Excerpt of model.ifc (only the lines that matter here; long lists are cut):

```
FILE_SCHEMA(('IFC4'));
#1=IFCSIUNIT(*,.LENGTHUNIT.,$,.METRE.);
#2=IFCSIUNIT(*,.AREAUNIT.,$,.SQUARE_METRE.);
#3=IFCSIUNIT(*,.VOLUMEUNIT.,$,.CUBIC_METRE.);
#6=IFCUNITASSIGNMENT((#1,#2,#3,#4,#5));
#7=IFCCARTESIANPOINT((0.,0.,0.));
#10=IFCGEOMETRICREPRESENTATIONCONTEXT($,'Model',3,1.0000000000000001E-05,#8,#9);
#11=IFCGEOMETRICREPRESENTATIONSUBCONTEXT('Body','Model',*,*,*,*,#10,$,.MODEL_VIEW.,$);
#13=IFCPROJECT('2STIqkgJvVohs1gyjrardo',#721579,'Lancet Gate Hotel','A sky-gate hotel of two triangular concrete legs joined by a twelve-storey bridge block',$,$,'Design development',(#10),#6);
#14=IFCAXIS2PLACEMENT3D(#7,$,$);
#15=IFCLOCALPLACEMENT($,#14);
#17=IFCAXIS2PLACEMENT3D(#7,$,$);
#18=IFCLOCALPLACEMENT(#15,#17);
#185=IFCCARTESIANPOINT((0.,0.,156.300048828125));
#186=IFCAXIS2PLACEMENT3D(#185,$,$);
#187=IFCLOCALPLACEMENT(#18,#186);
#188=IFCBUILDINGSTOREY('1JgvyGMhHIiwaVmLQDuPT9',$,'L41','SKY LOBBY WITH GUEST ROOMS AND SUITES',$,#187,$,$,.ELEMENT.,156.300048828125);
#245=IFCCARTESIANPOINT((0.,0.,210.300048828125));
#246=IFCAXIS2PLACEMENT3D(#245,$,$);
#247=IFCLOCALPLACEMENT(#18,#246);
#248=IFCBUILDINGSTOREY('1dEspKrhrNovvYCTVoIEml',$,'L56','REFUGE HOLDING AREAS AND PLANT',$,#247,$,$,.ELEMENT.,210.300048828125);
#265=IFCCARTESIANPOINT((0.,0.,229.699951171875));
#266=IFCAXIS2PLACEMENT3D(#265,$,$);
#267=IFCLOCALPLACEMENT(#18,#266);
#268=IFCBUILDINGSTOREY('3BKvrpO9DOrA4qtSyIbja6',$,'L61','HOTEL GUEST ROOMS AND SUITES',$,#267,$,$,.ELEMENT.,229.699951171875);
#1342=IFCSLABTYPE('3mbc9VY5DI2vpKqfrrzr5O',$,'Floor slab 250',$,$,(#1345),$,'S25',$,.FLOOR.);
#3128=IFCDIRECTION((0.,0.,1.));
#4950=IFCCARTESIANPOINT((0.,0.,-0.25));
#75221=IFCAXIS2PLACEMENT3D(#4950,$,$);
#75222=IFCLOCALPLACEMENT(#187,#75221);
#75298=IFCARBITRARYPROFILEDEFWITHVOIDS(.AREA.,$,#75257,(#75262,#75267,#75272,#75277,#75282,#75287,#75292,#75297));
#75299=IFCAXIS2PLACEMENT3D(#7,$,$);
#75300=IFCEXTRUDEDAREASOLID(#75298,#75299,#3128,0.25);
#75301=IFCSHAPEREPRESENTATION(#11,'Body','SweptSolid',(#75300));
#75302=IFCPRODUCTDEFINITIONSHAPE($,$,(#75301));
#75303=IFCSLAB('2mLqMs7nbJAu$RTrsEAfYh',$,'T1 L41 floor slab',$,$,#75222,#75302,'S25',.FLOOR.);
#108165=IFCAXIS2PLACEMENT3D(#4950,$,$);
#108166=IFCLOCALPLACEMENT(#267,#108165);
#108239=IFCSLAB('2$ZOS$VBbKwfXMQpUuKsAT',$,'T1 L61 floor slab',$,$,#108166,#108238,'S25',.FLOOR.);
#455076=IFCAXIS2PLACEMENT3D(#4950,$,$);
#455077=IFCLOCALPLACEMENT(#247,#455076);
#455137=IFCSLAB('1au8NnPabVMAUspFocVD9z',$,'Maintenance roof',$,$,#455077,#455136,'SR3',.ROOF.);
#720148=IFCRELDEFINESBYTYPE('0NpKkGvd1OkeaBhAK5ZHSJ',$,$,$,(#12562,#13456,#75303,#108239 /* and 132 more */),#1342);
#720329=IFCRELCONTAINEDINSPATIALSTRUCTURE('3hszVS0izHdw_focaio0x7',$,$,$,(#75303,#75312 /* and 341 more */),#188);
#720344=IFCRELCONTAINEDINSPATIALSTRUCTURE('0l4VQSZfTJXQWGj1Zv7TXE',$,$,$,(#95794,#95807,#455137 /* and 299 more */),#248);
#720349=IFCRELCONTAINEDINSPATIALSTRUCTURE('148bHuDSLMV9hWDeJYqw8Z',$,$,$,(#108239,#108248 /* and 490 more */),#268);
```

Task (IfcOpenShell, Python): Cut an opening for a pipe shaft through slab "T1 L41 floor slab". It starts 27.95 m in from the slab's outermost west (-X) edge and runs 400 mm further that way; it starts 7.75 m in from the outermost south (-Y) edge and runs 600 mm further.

```python
import numpy as np
import ifcopenshell
import ifcopenshell.api.feature
import ifcopenshell.api.geometry
import ifcopenshell.api.root
import ifcopenshell.geom
import ifcopenshell.util.placement
import ifcopenshell.util.representation
import ifcopenshell.util.shape
import ifcopenshell.util.unit

model = ifcopenshell.open("model.ifc")
unit_scale = ifcopenshell.util.unit.calculate_unit_scale(model)
settings = ifcopenshell.geom.settings()


def volume(element):
    """Net volume in cubic metres, openings subtracted."""
    shape = ifcopenshell.geom.create_shape(settings, element)
    return ifcopenshell.util.shape.get_volume(shape.geometry)


slab = model.by_id(75303)
before = volume(slab)

# Extent in the slab's own axes, in metres. The edges named are its -X and -Y sides.
slab_shape = ifcopenshell.geom.create_shape(settings, slab)
vertices = ifcopenshell.util.shape.get_vertices(slab_shape.geometry)
x_min, y_min, bottom = vertices.min(axis=0)
top = vertices[:, 2].max()

opening = ifcopenshell.api.root.create_entity(model, ifc_class="IfcOpeningElement", name="Pipe shaft opening", predefined_type="OPENING")
context = ifcopenshell.util.representation.get_context(model, "Model", "Body", "MODEL_VIEW")
width, depth = 0.4, 0.6
outline = [(0.0, 0.0), (width, 0.0), (width, depth), (0.0, depth), (0.0, 0.0)]
# Overshoot both faces by 50 mm so the cut is clean.
shape = ifcopenshell.api.geometry.add_slab_representation(
    model, context=context, depth=top - bottom + 0.1, polyline=outline
)
ifcopenshell.api.geometry.assign_representation(model, product=opening, representation=shape)

matrix = ifcopenshell.util.placement.get_local_placement(slab.ObjectPlacement)
matrix[:, 3] = matrix @ np.append(np.array([x_min + 27.95, y_min + 7.75, bottom - 0.05]) / unit_scale, 1.0)
ifcopenshell.api.geometry.edit_object_placement(model, product=opening, matrix=matrix, is_si=False)
ifcopenshell.api.feature.add_feature(model, feature=opening, element=slab)

after = volume(slab)

print(f"slab volume {before:.3f} -> {after:.3f} m3")

model.write("model_edited.ifc")
```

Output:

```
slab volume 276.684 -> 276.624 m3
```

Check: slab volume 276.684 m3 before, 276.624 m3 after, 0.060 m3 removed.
